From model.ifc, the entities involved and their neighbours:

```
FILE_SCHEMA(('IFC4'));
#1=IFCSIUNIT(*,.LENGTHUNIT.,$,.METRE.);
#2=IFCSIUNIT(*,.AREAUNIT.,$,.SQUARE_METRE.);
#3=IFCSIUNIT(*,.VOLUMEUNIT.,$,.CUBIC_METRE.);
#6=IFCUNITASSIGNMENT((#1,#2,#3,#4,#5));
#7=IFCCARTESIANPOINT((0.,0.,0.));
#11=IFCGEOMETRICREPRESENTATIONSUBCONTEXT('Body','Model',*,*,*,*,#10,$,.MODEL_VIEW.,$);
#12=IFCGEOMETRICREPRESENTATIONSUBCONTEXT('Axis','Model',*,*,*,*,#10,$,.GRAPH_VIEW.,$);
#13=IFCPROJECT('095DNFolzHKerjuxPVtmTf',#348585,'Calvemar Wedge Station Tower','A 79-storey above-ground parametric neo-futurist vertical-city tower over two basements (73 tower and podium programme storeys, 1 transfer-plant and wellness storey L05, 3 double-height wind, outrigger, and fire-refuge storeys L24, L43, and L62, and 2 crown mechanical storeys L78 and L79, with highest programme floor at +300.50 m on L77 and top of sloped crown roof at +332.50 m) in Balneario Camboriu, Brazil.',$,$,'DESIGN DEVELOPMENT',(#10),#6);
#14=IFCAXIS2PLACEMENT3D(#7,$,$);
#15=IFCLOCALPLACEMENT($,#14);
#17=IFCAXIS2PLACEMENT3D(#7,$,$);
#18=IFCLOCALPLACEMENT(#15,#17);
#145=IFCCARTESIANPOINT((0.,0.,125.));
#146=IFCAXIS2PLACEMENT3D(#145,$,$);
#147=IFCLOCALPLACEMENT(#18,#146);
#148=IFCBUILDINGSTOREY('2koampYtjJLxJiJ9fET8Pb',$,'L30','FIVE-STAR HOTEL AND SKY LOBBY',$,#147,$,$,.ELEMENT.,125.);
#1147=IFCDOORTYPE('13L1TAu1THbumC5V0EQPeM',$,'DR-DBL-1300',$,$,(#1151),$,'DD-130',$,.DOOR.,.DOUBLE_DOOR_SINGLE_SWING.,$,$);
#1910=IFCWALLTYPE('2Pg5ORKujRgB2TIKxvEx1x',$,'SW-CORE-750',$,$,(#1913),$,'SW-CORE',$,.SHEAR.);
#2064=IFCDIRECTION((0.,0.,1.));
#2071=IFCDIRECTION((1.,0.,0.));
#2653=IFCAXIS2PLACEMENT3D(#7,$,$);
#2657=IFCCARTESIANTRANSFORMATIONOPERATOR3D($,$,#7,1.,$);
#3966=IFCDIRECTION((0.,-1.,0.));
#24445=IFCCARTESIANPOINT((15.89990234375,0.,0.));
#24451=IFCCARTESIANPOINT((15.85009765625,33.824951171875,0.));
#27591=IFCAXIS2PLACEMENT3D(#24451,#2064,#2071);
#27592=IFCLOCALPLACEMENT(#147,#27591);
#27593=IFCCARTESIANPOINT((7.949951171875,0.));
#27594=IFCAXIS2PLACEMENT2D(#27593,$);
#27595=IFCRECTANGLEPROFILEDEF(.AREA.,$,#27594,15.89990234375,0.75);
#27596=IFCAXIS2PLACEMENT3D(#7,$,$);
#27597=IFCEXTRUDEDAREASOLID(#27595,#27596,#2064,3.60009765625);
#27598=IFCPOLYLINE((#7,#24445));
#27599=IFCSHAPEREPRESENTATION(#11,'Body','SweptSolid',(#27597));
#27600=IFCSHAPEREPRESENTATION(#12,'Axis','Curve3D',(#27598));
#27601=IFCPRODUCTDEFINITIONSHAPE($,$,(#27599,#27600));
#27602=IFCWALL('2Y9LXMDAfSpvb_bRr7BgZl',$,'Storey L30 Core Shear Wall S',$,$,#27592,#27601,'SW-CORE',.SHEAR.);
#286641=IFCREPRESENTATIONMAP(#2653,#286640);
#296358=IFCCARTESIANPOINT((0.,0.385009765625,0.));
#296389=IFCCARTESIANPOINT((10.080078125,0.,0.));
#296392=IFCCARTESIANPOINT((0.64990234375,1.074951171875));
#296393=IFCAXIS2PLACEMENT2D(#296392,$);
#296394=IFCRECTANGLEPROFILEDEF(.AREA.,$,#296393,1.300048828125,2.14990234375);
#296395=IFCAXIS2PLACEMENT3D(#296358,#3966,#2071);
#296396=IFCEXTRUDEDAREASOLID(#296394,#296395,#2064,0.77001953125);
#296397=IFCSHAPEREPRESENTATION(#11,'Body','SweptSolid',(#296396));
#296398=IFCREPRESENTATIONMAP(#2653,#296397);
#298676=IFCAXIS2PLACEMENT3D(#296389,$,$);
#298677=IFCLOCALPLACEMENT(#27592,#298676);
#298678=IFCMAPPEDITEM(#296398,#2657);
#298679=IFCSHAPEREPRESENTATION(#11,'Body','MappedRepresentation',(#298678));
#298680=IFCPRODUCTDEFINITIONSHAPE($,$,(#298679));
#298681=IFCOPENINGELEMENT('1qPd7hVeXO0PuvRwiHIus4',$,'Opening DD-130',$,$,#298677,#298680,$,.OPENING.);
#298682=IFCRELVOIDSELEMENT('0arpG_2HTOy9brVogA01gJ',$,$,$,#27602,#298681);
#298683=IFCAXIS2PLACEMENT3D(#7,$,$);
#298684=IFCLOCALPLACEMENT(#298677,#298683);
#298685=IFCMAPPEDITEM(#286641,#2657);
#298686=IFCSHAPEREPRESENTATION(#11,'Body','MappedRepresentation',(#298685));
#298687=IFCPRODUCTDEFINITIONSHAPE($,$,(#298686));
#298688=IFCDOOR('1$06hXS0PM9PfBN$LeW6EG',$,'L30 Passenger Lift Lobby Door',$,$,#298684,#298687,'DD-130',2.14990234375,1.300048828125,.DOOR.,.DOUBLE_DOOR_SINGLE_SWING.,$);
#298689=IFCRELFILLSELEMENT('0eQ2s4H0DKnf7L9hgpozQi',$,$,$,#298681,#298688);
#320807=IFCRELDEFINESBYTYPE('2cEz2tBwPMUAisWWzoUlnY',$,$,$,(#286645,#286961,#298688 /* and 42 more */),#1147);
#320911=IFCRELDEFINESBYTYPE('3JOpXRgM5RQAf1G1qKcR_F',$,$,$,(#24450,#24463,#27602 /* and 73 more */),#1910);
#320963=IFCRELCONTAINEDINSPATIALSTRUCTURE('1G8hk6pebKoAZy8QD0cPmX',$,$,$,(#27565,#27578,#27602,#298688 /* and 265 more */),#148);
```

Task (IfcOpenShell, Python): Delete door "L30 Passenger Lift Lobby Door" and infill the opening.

```python
import ifcopenshell
import ifcopenshell.api.feature
import ifcopenshell.api.root
import ifcopenshell.geom
import ifcopenshell.util.shape

model = ifcopenshell.open("model.ifc")
settings = ifcopenshell.geom.settings()


def volume(element):
    """Net volume in cubic metres, openings subtracted."""
    shape = ifcopenshell.geom.create_shape(settings, element)
    return ifcopenshell.util.shape.get_volume(shape.geometry)


door = model.by_guid("1$06hXS0PM9PfBN$LeW6EG")
opening = door.FillsVoids[0].RelatingOpeningElement
wall = opening.VoidsElements[0].RelatingBuildingElement
before = volume(wall)

ifcopenshell.api.root.remove_product(model, product=door)
ifcopenshell.api.feature.remove_feature(model, feature=opening)

after = volume(wall)

print(f"wall volume {before:.3f} -> {after:.3f} m3")

model.write("model_v2.ifc")
```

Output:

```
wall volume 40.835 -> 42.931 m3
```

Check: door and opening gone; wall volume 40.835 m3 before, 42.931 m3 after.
